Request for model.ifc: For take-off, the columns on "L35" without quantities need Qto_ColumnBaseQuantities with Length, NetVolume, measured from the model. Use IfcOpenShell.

First a look at what the model holds.

```python
import ifcopenshell
import ifcopenshell.util.element
import ifcopenshell.util.unit

model = ifcopenshell.open("model.ifc")
print(model.schema)
for unit_type in ("LENGTHUNIT", "AREAUNIT", "VOLUMEUNIT"):
    print(unit_type, ifcopenshell.util.unit.calculate_unit_scale(model, unit_type))
storey = next(s for s in model.by_type("IfcBuildingStorey") if s.Name == "L35")
columns = [e for e in ifcopenshell.util.element.get_decomposition(storey) if e.is_a("IfcColumn")]
for e in sorted(columns, key=lambda e: e.id()):
    print(e.id(), e.is_a(), e.Name, list(ifcopenshell.util.element.get_psets(e, qtos_only=True)), sep=" | ")
```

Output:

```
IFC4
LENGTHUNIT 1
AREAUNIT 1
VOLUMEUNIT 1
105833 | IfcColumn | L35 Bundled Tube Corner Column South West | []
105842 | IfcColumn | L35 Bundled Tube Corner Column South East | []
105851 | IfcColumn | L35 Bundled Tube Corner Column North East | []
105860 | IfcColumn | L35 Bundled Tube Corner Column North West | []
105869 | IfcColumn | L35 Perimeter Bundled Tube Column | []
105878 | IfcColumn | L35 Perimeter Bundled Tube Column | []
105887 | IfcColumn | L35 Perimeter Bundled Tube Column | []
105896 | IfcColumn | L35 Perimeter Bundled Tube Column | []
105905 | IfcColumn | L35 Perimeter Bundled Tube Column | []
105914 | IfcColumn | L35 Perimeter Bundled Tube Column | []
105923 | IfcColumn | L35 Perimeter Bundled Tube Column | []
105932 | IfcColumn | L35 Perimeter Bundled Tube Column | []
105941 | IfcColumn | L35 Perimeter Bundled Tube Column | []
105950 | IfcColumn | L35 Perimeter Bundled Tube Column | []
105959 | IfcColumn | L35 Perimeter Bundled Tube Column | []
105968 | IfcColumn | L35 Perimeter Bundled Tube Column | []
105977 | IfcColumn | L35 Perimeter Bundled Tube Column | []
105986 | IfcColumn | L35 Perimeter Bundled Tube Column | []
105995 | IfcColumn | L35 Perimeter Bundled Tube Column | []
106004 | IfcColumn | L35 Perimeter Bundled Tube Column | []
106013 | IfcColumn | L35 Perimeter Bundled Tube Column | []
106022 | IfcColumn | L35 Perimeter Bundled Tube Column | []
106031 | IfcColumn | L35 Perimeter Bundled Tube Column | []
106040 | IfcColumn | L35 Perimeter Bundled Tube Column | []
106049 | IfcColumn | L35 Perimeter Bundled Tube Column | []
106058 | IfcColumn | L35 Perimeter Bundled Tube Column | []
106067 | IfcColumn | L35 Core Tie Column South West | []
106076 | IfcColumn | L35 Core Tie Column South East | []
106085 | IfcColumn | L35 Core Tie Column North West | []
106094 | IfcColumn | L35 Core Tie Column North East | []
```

```python
import ifcopenshell
import ifcopenshell.api.pset
import ifcopenshell.geom
import ifcopenshell.util.element
import ifcopenshell.util.shape
import ifcopenshell.util.unit

model = ifcopenshell.open("model.ifc")
unit_scale = ifcopenshell.util.unit.calculate_unit_scale(model)
volume_scale = ifcopenshell.util.unit.calculate_unit_scale(model, "VOLUMEUNIT")
settings = ifcopenshell.geom.settings()

storey = next(s for s in model.by_type("IfcBuildingStorey") if s.Name == "L35")
columns = [e for e in ifcopenshell.util.element.get_decomposition(storey) if e.is_a("IfcColumn")]

for e in sorted(columns, key=lambda e: e.id()):
    if ifcopenshell.util.element.get_psets(e, qtos_only=True, should_inherit=False):
        continue
    # Geometry comes back in metres, in the element's own axes.
    shape = ifcopenshell.geom.create_shape(settings, e)
    values = {
        "Length": ifcopenshell.util.shape.get_z(shape.geometry) / unit_scale,
        "NetVolume": ifcopenshell.util.shape.get_volume(shape.geometry) / volume_scale,
    }
    qto = ifcopenshell.api.pset.add_qto(model, product=e, name="Qto_ColumnBaseQuantities")
    ifcopenshell.api.pset.edit_qto(model, qto=qto, properties=values)
    print(e.id(), {k: round(v, 3) for k, v in values.items()})

model.write("model_edited.ifc")
```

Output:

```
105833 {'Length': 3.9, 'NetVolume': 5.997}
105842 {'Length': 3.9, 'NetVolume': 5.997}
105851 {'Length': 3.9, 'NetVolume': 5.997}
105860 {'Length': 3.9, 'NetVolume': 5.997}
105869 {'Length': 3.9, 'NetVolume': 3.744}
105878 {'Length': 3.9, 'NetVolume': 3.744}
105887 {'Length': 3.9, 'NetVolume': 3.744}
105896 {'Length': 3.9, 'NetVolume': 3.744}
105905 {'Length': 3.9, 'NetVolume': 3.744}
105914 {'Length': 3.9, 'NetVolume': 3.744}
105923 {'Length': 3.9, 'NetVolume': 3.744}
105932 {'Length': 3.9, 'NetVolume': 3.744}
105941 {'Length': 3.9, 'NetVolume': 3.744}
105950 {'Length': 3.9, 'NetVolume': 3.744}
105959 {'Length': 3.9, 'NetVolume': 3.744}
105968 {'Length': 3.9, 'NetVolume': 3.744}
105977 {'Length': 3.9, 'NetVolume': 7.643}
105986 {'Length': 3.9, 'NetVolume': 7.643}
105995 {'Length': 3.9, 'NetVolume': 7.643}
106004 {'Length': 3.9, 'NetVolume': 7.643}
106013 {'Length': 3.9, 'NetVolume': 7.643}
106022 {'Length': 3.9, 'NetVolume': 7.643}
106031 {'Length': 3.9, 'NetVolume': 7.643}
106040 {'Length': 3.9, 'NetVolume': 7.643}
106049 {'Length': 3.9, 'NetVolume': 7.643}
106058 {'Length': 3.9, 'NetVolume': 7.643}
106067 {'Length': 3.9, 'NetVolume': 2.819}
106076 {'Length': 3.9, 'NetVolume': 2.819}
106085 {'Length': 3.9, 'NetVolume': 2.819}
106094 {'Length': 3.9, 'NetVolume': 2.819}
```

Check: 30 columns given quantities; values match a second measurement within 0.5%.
